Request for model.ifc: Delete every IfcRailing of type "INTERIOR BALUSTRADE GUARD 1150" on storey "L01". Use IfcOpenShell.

First a look at what the model holds.

```python
import ifcopenshell
import ifcopenshell.util.element

model = ifcopenshell.open("model.ifc")
print(model.schema)
storey = next(s for s in model.by_type("IfcBuildingStorey") if s.Name == "L01")
railings = [e for e in ifcopenshell.util.element.get_decomposition(storey) if e.is_a("IfcRailing")]
seen = {}
for e in railings:
    element_type = ifcopenshell.util.element.get_type(e)
    name = element_type.Name if element_type not in (None, e) else None
    seen[name] = seen.get(name, 0) + 1
for name, count in sorted(seen.items(), key=str):
    print(count, "x", name)
```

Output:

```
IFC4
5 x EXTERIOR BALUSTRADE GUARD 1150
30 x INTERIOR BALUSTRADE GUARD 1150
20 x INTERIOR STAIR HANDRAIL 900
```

```python
import ifcopenshell
import ifcopenshell.api.root
import ifcopenshell.util.element

model = ifcopenshell.open("model.ifc")

storey = next(s for s in model.by_type("IfcBuildingStorey") if s.Name == "L01")
railings = [e for e in ifcopenshell.util.element.get_decomposition(storey) if e.is_a("IfcRailing")]
targets = [e for e in railings if (t := ifcopenshell.util.element.get_type(e)) not in (None, e) and t.Name == "INTERIOR BALUSTRADE GUARD 1150"]

for e in targets:
    ifcopenshell.api.root.remove_product(model, product=e)
print(len(targets), "removed")

model.write("model_rev.ifc")
```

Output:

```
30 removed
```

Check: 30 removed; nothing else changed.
